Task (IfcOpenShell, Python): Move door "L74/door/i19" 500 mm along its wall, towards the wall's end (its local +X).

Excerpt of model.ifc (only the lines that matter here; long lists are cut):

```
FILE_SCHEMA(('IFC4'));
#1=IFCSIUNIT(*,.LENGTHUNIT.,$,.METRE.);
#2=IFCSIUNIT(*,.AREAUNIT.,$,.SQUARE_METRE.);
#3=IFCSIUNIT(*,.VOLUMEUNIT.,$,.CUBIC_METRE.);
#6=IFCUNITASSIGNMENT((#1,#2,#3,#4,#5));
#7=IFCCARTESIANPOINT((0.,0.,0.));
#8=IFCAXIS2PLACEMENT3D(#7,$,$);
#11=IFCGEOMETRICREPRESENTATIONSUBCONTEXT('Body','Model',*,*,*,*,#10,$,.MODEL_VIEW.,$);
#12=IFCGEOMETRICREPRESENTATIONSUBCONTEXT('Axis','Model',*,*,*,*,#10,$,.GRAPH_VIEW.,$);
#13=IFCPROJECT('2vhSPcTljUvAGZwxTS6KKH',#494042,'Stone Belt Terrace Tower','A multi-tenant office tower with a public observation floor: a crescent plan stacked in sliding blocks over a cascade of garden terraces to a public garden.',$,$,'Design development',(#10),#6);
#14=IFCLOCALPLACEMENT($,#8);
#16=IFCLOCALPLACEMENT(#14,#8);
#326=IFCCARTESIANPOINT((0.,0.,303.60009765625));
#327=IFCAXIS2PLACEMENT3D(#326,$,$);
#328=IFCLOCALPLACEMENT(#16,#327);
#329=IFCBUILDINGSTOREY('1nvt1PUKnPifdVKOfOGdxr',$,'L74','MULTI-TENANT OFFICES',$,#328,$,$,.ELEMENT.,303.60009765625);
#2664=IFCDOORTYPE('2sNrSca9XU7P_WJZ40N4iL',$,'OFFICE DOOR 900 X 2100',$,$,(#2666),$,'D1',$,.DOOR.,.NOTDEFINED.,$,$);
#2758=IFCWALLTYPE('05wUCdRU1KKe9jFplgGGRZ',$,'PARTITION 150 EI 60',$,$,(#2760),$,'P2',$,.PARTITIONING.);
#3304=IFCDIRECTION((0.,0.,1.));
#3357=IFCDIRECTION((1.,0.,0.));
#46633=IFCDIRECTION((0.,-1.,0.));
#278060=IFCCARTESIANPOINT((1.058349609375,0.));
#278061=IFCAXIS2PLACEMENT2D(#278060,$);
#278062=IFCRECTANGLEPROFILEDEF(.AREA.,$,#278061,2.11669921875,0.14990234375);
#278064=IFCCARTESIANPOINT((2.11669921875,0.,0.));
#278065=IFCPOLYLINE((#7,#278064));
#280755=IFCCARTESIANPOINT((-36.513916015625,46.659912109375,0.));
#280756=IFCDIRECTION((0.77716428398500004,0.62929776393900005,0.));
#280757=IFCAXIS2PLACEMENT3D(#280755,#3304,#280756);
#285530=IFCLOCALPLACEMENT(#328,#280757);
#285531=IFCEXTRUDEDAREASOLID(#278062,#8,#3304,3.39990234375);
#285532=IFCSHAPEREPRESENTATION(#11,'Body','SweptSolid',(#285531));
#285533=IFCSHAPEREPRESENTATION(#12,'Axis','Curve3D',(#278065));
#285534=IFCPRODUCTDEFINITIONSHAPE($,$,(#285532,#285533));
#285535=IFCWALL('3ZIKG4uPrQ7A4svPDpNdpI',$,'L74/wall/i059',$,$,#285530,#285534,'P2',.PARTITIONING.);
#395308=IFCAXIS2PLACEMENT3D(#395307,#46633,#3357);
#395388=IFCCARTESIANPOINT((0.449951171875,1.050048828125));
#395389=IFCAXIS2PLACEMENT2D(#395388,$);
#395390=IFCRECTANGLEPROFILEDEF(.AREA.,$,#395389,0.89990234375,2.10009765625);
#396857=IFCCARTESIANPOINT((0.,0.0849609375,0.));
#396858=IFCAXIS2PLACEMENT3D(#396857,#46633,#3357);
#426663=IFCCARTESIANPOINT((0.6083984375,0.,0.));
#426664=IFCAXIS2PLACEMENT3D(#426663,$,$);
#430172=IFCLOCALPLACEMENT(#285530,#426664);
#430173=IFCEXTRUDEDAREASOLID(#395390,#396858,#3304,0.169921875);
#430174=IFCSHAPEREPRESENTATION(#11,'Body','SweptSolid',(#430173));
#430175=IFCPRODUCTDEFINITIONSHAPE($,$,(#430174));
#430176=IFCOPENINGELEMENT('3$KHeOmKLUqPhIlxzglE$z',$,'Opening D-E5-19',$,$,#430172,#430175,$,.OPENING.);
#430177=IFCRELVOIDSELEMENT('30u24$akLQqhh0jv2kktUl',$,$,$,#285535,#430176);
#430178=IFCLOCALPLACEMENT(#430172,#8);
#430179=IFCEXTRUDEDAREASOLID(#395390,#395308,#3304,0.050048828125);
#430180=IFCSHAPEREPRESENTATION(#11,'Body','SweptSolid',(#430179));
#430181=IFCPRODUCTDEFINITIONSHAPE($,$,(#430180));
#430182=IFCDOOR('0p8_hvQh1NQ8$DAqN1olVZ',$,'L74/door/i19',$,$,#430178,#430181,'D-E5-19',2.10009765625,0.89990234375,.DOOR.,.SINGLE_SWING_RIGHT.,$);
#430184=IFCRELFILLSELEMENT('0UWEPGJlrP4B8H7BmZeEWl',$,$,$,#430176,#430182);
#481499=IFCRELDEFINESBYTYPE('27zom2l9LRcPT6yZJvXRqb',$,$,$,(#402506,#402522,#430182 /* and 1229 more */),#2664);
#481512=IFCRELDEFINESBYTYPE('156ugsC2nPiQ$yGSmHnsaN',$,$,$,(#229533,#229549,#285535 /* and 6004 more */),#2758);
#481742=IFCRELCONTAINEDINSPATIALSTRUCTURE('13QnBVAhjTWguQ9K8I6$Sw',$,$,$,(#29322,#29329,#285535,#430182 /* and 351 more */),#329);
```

```python
import ifcopenshell
import ifcopenshell.api.geometry
import ifcopenshell.util.placement

model = ifcopenshell.open("model.ifc")

door = model.by_id(430182)
opening = door.FillsVoids[0].RelatingOpeningElement
wall = opening.VoidsElements[0].RelatingBuildingElement

wall_matrix = ifcopenshell.util.placement.get_local_placement(wall.ObjectPlacement)
shift = wall_matrix[:3, 0] * 0.5
before = ifcopenshell.util.placement.get_local_placement(door.ObjectPlacement)[:3, 3].copy()

# The door is placed relative to its opening, so it follows when the opening moves.
matrix = ifcopenshell.util.placement.get_local_placement(opening.ObjectPlacement)
matrix[:3, 3] += shift
ifcopenshell.api.geometry.edit_object_placement(
    model, product=opening, matrix=matrix, is_si=False, should_transform_children=True
)

after = ifcopenshell.util.placement.get_local_placement(door.ObjectPlacement)[:3, 3]
print("door moved by", (after - before).round(3) + 0.0)

model.write("model-out.ifc")
```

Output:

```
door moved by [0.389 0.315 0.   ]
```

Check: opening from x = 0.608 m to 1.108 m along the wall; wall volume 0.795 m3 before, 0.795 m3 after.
